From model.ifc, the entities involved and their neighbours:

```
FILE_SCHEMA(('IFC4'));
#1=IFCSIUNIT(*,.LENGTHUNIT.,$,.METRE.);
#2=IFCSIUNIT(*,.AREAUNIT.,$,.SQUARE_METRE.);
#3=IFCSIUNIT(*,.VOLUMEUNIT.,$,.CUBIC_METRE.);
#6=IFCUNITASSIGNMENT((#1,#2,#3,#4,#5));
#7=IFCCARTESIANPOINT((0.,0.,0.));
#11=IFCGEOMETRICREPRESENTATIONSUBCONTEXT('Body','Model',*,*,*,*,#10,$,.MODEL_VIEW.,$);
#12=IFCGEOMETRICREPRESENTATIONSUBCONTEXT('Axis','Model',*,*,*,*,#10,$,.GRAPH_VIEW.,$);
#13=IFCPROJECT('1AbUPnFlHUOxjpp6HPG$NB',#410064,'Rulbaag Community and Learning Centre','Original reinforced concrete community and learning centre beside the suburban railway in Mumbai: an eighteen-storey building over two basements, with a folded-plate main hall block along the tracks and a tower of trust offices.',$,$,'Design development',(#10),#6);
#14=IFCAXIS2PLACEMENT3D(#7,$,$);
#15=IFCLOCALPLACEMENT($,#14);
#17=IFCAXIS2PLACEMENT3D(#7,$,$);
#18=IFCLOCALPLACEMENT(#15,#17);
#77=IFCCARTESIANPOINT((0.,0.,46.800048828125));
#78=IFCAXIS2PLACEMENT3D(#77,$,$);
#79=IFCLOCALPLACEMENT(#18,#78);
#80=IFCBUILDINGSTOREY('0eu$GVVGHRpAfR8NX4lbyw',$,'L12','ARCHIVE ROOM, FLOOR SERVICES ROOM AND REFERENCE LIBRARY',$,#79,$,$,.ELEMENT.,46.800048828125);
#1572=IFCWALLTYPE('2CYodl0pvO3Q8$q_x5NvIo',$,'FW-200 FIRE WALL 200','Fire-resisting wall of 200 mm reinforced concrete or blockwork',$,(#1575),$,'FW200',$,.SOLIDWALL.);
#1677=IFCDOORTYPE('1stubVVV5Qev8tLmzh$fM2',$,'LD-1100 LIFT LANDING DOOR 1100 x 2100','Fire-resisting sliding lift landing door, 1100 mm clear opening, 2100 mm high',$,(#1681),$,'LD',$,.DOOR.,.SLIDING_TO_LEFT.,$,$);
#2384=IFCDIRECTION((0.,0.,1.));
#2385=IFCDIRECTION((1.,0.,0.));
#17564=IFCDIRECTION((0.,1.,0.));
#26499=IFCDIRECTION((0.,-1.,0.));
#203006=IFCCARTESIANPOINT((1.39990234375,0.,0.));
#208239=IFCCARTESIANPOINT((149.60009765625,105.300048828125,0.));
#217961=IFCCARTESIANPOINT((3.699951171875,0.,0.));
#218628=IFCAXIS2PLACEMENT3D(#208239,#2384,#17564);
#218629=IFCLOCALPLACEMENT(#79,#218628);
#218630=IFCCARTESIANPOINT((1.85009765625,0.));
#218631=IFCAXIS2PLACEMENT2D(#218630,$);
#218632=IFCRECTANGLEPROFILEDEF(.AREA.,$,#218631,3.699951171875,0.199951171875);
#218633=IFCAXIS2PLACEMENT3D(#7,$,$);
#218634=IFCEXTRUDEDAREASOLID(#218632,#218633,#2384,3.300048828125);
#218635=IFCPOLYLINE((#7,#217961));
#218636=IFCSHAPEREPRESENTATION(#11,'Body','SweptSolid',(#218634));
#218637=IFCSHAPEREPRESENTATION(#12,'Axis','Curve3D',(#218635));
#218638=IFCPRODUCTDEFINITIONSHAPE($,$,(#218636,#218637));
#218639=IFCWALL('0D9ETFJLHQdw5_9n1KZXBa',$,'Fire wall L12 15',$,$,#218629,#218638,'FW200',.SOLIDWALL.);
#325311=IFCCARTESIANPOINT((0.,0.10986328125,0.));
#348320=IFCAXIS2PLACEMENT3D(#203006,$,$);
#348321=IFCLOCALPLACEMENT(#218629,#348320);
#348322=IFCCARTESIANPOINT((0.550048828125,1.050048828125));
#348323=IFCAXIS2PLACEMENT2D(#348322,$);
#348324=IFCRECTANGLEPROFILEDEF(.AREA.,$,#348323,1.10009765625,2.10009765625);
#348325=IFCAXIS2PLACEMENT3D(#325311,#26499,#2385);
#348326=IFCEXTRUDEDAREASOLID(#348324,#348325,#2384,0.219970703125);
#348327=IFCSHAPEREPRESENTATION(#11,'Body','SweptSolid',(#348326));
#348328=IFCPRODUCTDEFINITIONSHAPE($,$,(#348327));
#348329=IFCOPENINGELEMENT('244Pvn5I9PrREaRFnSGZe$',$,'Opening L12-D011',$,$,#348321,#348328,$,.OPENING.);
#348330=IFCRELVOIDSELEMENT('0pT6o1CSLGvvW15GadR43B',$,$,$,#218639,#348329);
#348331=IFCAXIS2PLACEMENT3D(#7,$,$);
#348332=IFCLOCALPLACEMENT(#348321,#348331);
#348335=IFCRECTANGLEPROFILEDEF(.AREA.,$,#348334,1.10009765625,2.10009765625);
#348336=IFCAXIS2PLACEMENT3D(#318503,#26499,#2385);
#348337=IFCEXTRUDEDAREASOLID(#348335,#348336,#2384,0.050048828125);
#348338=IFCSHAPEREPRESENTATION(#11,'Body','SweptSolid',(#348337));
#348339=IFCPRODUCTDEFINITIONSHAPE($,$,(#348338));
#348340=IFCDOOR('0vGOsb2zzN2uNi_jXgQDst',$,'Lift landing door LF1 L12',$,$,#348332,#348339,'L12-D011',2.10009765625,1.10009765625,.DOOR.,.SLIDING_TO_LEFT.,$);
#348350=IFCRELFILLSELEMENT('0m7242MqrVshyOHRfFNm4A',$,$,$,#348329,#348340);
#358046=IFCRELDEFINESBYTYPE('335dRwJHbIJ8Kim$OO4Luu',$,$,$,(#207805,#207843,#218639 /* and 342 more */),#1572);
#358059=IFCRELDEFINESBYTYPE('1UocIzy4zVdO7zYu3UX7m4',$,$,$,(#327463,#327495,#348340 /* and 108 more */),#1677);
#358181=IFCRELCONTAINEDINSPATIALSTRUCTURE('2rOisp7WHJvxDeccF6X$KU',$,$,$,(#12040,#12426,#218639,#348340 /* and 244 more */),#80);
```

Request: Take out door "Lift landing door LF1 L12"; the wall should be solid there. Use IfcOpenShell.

```python
import ifcopenshell
import ifcopenshell.api.feature
import ifcopenshell.api.root
import ifcopenshell.geom
import ifcopenshell.util.shape

model = ifcopenshell.open("model.ifc")
settings = ifcopenshell.geom.settings()


def volume(element):
    """Net volume in cubic metres, openings subtracted."""
    shape = ifcopenshell.geom.create_shape(settings, element)
    return ifcopenshell.util.shape.get_volume(shape.geometry)


door = model.by_id(348340)
opening = door.FillsVoids[0].RelatingOpeningElement
wall = opening.VoidsElements[0].RelatingBuildingElement
before = volume(wall)

ifcopenshell.api.root.remove_product(model, product=door)
ifcopenshell.api.feature.remove_feature(model, feature=opening)

after = volume(wall)

print(f"wall volume {before:.3f} -> {after:.3f} m3")

model.write("model_edited.ifc")
```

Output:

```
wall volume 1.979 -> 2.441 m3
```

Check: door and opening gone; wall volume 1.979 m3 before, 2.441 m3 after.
